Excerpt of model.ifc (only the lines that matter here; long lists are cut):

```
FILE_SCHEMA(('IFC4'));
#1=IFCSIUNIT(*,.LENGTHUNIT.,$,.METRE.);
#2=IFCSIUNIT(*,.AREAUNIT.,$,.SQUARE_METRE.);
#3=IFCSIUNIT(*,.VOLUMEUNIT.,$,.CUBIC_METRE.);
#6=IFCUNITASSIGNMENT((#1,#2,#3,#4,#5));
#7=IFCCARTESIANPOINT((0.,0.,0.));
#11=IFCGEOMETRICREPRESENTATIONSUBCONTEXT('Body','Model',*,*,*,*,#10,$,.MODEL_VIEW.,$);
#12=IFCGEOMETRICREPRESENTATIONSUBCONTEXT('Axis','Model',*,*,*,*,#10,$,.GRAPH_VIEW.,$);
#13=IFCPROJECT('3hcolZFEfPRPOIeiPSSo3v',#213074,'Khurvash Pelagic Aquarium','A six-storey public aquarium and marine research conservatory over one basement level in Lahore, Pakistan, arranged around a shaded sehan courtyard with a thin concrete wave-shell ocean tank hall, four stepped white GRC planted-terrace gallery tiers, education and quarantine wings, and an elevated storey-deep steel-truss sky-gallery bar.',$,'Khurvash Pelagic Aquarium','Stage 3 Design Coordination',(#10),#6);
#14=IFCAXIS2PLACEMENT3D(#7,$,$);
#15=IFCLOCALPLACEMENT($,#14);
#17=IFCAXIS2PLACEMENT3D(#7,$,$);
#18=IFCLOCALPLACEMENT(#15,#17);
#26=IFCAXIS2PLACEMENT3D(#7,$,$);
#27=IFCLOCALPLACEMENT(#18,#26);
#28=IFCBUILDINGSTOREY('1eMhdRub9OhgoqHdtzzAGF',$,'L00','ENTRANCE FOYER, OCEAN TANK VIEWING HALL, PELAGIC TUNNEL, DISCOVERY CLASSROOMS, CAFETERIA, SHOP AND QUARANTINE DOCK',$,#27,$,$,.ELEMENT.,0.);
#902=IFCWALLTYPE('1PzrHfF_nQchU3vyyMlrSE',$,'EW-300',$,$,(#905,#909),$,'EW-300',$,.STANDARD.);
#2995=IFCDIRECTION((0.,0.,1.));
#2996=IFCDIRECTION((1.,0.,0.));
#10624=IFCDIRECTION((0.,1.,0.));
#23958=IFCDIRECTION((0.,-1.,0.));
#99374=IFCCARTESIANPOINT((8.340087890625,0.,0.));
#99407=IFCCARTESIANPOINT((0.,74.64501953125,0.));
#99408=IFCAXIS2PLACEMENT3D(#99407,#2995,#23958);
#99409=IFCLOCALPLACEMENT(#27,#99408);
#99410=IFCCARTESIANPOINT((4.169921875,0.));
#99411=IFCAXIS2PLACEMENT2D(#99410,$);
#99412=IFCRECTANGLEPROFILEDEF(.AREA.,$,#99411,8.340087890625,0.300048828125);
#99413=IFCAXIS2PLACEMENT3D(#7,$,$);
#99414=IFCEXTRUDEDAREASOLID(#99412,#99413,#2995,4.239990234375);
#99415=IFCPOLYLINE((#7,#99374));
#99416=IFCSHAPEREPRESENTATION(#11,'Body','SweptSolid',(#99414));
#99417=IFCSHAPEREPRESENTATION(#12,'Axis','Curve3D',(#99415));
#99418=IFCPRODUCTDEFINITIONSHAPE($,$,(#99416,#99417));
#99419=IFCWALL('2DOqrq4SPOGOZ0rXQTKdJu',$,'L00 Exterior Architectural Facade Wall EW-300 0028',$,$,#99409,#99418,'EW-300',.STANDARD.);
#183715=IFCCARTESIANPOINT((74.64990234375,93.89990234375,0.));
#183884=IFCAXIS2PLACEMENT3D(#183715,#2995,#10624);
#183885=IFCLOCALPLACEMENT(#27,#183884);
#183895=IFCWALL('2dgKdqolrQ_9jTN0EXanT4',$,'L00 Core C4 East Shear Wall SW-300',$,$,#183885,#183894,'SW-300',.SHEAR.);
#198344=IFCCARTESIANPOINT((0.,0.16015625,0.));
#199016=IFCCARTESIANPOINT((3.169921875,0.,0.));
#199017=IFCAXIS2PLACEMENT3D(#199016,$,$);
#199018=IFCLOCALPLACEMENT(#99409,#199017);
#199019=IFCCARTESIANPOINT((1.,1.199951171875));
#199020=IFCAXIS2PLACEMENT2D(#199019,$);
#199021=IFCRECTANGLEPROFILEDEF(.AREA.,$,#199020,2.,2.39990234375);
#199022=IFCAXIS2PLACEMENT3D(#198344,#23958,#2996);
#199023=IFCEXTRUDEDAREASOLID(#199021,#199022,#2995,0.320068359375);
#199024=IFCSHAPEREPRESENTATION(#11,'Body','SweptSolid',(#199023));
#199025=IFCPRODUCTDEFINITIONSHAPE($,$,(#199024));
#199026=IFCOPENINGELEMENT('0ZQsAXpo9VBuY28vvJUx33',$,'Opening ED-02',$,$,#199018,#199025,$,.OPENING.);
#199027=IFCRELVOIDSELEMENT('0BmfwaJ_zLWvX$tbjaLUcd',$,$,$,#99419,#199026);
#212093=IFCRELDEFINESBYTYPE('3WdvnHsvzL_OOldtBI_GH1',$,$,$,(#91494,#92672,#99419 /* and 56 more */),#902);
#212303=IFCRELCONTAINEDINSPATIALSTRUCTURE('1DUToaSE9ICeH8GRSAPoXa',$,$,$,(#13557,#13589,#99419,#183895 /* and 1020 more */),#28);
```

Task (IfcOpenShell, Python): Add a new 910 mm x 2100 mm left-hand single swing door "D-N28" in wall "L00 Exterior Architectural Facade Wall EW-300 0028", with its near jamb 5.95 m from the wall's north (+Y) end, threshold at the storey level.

```python
import numpy as np
import ifcopenshell
import ifcopenshell.api.feature
import ifcopenshell.api.geometry
import ifcopenshell.api.root
import ifcopenshell.api.spatial
import ifcopenshell.geom
import ifcopenshell.util.element
import ifcopenshell.util.placement
import ifcopenshell.util.representation
import ifcopenshell.util.shape
import ifcopenshell.util.unit

model = ifcopenshell.open("model.ifc")
unit_scale = ifcopenshell.util.unit.calculate_unit_scale(model)
settings = ifcopenshell.geom.settings()


def volume(element):
    """Net volume in cubic metres, openings subtracted."""
    shape = ifcopenshell.geom.create_shape(settings, element)
    return ifcopenshell.util.shape.get_volume(shape.geometry)


wall = model.by_guid("2DOqrq4SPOGOZ0rXQTKdJu")
storey = ifcopenshell.util.element.get_container(wall, ifc_class="IfcBuildingStorey")
context = ifcopenshell.util.representation.get_context(model, "Model", "Body", "MODEL_VIEW")
before = volume(wall)

width, height, from_end, sill = 0.91, 2.1, 5.95, 0.0  # metres

# The wall runs along its own X axis, and the end named is its -X end.
wall_shape = ifcopenshell.geom.create_shape(settings, wall)
x, y, z = ifcopenshell.util.shape.get_vertices(wall_shape.geometry).T
start = x.min() + from_end
face, thickness = float(y.min()), float(y.max() - y.min())
wall_matrix = ifcopenshell.util.placement.get_local_placement(wall.ObjectPlacement)
level = ifcopenshell.util.placement.get_local_placement(storey.ObjectPlacement)[2, 3]


def in_wall(x, y):
    """Placement at x, y metres in the wall's axes, at sill height."""
    matrix = wall_matrix.copy()
    matrix[:, 3] = wall_matrix @ np.array([x / unit_scale, y / unit_scale, 0.0, 1.0])
    matrix[2, 3] = level + sill / unit_scale
    return matrix


# Opening: a box that overshoots both wall faces by 50 mm.
opening = ifcopenshell.api.root.create_entity(model, ifc_class="IfcOpeningElement", predefined_type="OPENING")
box = ifcopenshell.api.geometry.add_wall_representation(
    model, context=context, length=width, height=height, thickness=thickness + 0.1
)
ifcopenshell.api.geometry.assign_representation(model, product=opening, representation=box)
ifcopenshell.api.geometry.edit_object_placement(model, product=opening, matrix=in_wall(start, face - 0.05), is_si=False)
ifcopenshell.api.feature.add_feature(model, feature=opening, element=wall)

door = ifcopenshell.api.root.create_entity(model, ifc_class="IfcDoor", name="D-N28", predefined_type="DOOR")
door.OverallWidth, door.OverallHeight = width / unit_scale, height / unit_scale
door.OperationType = "SINGLE_SWING_LEFT"
body = ifcopenshell.api.geometry.add_door_representation(
    model,
    context=context,
    overall_width=door.OverallWidth,
    overall_height=door.OverallHeight,
    operation_type="SINGLE_SWING_LEFT",
    lining_properties={"LiningDepth": thickness / unit_scale, "ThresholdDepth": thickness / unit_scale},
)
ifcopenshell.api.geometry.assign_representation(model, product=door, representation=body)
ifcopenshell.api.spatial.assign_container(model, products=[door], relating_structure=storey)
ifcopenshell.api.feature.add_filling(model, opening=opening, element=door)

# The lining spans the wall, so the door starts at the wall face.
ifcopenshell.api.geometry.edit_object_placement(model, product=door, matrix=in_wall(start, face), is_si=False)

after = volume(wall)

print(f"wall volume {before:.3f} -> {after:.3f} m3")

model.write("model-out.ifc")
```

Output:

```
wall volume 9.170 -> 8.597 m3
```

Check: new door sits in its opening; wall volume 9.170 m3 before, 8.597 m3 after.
